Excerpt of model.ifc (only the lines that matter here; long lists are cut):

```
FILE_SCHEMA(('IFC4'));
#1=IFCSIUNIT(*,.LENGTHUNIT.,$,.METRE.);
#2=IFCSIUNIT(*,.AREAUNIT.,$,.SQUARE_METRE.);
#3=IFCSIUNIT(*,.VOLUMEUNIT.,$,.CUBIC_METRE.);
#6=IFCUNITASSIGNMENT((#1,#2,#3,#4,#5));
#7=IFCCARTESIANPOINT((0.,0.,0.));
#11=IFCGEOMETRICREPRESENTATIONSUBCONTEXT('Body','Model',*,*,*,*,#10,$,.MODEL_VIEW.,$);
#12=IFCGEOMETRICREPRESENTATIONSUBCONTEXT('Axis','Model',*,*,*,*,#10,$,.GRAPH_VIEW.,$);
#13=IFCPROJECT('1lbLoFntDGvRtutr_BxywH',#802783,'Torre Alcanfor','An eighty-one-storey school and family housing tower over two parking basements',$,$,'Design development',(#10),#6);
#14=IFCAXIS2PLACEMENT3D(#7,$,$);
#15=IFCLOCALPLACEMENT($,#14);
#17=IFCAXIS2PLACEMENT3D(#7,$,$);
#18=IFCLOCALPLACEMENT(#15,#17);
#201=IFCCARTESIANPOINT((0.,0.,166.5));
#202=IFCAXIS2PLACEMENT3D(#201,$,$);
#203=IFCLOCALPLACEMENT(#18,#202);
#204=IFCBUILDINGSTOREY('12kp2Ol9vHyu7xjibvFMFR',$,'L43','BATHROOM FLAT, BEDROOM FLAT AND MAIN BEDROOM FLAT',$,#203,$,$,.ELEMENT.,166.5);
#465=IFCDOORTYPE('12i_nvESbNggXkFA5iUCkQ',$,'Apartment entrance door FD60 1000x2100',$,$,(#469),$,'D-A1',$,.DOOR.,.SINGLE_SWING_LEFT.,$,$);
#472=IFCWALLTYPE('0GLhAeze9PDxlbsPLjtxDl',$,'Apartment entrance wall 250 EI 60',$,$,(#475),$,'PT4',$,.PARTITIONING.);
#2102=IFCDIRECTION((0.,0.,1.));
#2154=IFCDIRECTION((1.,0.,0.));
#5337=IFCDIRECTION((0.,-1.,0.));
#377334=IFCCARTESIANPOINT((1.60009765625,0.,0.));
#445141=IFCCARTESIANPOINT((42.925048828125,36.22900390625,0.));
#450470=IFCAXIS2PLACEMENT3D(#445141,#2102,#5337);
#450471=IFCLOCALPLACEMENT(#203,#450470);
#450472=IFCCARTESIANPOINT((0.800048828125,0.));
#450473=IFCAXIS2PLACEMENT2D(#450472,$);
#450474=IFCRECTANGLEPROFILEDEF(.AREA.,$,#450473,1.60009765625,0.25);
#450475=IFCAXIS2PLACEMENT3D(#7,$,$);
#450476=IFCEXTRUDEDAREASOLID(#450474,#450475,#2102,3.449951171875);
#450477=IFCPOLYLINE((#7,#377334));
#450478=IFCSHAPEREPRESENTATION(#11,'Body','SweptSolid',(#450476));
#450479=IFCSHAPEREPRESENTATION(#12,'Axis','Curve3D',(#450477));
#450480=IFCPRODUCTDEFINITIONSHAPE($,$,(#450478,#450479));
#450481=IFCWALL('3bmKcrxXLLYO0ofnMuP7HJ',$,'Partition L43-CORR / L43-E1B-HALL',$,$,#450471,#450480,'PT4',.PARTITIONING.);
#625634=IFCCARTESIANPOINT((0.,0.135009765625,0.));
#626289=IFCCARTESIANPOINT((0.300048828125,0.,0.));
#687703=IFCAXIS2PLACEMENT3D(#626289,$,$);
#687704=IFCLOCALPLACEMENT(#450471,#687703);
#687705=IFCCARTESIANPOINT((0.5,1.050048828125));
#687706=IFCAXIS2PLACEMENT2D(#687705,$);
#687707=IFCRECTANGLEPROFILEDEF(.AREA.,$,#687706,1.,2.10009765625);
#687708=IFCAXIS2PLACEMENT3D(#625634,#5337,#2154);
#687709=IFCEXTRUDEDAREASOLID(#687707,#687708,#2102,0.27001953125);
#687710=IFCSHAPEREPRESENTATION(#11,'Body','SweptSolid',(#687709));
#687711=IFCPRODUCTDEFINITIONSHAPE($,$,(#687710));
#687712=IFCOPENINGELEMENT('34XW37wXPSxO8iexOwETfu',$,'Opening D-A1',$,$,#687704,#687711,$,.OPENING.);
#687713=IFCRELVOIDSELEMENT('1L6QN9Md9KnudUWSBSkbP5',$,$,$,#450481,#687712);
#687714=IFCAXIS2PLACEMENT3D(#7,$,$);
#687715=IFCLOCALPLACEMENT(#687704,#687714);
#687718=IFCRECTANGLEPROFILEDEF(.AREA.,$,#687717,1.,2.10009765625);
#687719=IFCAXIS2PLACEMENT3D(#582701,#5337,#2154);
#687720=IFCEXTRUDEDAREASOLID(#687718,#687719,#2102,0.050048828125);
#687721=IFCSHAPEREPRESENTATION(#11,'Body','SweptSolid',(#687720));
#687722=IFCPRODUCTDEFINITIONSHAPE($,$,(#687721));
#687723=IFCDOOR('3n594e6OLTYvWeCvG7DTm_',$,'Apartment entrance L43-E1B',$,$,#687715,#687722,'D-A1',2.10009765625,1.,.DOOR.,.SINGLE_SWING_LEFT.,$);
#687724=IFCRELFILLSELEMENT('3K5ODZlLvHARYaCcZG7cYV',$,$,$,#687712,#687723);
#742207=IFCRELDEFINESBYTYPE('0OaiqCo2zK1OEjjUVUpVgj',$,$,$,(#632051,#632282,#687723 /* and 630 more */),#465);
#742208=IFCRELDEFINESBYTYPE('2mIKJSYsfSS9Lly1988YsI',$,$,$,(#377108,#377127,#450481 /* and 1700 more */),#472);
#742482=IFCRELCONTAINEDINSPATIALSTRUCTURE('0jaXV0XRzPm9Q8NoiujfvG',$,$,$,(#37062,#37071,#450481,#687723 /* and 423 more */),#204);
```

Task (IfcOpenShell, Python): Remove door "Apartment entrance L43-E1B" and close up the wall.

```python
import ifcopenshell
import ifcopenshell.api.feature
import ifcopenshell.api.root
import ifcopenshell.geom
import ifcopenshell.util.shape

model = ifcopenshell.open("model.ifc")
settings = ifcopenshell.geom.settings()


def volume(element):
    """Net volume in cubic metres, openings subtracted."""
    shape = ifcopenshell.geom.create_shape(settings, element)
    return ifcopenshell.util.shape.get_volume(shape.geometry)


door = model.by_guid("3n594e6OLTYvWeCvG7DTm_")
opening = door.FillsVoids[0].RelatingOpeningElement
wall = opening.VoidsElements[0].RelatingBuildingElement
before = volume(wall)

ifcopenshell.api.root.remove_product(model, product=door)
ifcopenshell.api.feature.remove_feature(model, feature=opening)

after = volume(wall)

print(f"wall volume {before:.3f} -> {after:.3f} m3")

model.write("model_rev.ifc")
```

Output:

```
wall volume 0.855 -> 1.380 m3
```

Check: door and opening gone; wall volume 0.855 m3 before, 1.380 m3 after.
